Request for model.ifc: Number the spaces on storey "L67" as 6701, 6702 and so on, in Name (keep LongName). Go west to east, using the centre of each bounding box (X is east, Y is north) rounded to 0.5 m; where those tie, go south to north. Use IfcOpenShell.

First a look at what the model holds.

```python
import ifcopenshell
import ifcopenshell.util.element
import ifcopenshell.util.placement

model = ifcopenshell.open("model.ifc")
print(model.schema)
storey = next(s for s in model.by_type("IfcBuildingStorey") if s.Name == "L67")
spaces = [e for e in ifcopenshell.util.element.get_decomposition(storey) if e.is_a("IfcSpace")]
for e in sorted(spaces, key=lambda e: e.id()):
    origin = ifcopenshell.util.placement.get_local_placement(e.ObjectPlacement)[:3, 3]
    print(e.id(), e.Name, e.LongName, origin.round(2) + 0.0, sep=" | ")
```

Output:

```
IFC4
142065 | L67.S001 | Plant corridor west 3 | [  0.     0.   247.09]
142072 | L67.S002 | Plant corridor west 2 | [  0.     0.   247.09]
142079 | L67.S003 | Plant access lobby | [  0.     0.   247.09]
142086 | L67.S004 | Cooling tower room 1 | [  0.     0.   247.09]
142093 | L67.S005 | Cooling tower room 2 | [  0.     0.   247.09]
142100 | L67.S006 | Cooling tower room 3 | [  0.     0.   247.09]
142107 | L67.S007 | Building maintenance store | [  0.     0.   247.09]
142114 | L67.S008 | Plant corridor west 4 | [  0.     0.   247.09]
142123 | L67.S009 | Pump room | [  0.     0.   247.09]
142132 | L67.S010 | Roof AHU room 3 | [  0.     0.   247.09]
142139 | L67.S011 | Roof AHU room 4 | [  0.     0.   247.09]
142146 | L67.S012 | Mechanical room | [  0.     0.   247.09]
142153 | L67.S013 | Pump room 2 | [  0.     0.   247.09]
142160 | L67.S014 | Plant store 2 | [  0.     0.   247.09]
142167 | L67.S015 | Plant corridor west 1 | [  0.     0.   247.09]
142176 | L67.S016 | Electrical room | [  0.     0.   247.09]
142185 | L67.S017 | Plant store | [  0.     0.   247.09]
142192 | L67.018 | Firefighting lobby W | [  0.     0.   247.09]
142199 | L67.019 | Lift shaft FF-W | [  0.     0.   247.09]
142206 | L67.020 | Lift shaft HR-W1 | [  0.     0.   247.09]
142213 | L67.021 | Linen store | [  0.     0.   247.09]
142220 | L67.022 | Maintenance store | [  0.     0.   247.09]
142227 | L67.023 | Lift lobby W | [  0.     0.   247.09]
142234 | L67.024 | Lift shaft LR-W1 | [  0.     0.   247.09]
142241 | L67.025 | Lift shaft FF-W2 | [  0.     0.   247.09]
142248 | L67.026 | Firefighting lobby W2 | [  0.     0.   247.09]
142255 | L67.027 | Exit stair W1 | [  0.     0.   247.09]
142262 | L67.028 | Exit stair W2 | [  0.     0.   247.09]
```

```python
import ifcopenshell
import ifcopenshell.geom
import ifcopenshell.util.element
import ifcopenshell.util.shape

model = ifcopenshell.open("model.ifc")
settings = ifcopenshell.geom.settings()
settings.set("use-world-coords", True)


def centre(element):
    shape = ifcopenshell.geom.create_shape(settings, element)
    return ifcopenshell.util.shape.get_bbox_centroid(shape.geometry)


storey = next(s for s in model.by_type("IfcBuildingStorey") if s.Name == "L67")
spaces = [e for e in ifcopenshell.util.element.get_decomposition(storey) if e.is_a("IfcSpace")]

# Insertion points can sit at a corner or the storey origin, so sort by the geometry (in metres).
centres = {e: centre(e) for e in spaces}
spaces.sort(key=lambda e: (round(centres[e][0] / 0.5), centres[e][1]))

for i, e in enumerate(spaces, start=1):
    number = f"67{i:02d}"
    e.Name = number
    print(e.id(), number)

model.write("model_updated.ifc")
```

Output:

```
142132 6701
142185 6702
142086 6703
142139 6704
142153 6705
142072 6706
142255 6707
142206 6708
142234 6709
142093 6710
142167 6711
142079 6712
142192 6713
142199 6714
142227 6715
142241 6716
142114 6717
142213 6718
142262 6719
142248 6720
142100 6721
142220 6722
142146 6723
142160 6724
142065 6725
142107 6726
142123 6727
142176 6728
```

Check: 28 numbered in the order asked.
